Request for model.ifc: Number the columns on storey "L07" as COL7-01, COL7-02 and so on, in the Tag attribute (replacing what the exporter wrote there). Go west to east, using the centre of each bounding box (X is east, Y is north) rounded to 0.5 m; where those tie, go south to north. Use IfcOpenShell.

First a look at what the model holds.

```python
import ifcopenshell
import ifcopenshell.util.element
import ifcopenshell.util.placement

model = ifcopenshell.open("model.ifc")
print(model.schema)
storey = next(s for s in model.by_type("IfcBuildingStorey") if s.Name == "L07")
columns = [e for e in ifcopenshell.util.element.get_decomposition(storey) if e.is_a("IfcColumn")]
for e in sorted(columns, key=lambda e: e.id()):
    origin = ifcopenshell.util.placement.get_local_placement(e.ObjectPlacement)[:3, 3]
    print(e.id(), e.Tag, e.Name, origin.round(2) + 0.0, sep=" | ")
```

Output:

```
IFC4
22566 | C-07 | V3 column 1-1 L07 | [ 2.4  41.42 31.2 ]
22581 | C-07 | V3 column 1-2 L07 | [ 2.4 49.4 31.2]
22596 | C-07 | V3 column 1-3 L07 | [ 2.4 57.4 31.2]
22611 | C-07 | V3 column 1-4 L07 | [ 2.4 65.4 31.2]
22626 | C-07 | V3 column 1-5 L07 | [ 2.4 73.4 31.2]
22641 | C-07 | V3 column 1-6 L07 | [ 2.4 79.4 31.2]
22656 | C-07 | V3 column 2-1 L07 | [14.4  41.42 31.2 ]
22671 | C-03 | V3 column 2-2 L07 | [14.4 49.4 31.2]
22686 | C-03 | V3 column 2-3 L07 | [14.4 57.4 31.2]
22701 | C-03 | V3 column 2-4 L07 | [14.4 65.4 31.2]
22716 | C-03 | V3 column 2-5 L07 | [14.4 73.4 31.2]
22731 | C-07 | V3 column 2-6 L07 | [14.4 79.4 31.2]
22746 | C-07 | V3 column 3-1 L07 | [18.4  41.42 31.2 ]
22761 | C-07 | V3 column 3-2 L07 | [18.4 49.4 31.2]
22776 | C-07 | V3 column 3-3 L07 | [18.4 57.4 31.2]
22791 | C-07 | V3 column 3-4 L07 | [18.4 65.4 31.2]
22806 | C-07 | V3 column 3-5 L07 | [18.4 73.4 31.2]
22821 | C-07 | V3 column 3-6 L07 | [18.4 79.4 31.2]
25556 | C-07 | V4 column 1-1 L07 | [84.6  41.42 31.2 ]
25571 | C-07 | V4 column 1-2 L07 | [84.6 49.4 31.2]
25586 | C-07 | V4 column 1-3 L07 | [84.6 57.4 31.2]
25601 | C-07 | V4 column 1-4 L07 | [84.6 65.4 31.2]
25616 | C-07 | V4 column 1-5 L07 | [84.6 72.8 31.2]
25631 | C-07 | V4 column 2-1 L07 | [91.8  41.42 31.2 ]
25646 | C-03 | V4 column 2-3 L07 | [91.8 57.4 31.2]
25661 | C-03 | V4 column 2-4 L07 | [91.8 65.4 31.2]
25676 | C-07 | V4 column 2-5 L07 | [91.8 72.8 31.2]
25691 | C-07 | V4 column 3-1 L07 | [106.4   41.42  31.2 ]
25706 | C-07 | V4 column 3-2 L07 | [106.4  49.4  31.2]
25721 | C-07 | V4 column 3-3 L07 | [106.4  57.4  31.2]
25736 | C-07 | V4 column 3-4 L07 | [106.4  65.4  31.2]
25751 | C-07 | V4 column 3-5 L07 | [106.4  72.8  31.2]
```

```python
import ifcopenshell
import ifcopenshell.geom
import ifcopenshell.util.element
import ifcopenshell.util.shape

model = ifcopenshell.open("model.ifc")
settings = ifcopenshell.geom.settings()
settings.set("use-world-coords", True)


def centre(element):
    shape = ifcopenshell.geom.create_shape(settings, element)
    return ifcopenshell.util.shape.get_bbox_centroid(shape.geometry)


storey = next(s for s in model.by_type("IfcBuildingStorey") if s.Name == "L07")
columns = [e for e in ifcopenshell.util.element.get_decomposition(storey) if e.is_a("IfcColumn")]

# Insertion points can sit at a corner or the storey origin, so sort by the geometry (in metres).
centres = {e: centre(e) for e in columns}
columns.sort(key=lambda e: (round(centres[e][0] / 0.5), centres[e][1]))

for i, e in enumerate(columns, start=1):
    number = f"COL7-{i:02d}"
    e.Tag = number
    print(e.id(), number)

model.write("model_updated.ifc")
```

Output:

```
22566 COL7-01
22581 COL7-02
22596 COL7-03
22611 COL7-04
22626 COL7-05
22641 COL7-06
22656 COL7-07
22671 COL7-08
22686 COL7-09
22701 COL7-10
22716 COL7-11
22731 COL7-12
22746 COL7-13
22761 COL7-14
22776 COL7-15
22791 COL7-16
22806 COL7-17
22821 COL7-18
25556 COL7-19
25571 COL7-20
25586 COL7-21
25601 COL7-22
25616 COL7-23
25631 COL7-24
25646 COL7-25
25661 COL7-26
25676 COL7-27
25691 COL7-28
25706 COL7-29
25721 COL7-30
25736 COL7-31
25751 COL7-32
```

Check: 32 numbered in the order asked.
